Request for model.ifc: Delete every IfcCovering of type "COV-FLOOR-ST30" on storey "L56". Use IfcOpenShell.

First a look at what the model holds.

```python
import ifcopenshell
import ifcopenshell.util.element

model = ifcopenshell.open("model.ifc")
print(model.schema)
storey = next(s for s in model.by_type("IfcBuildingStorey") if s.Name == "L56")
coverings = [e for e in ifcopenshell.util.element.get_decomposition(storey) if e.is_a("IfcCovering")]
seen = {}
for e in coverings:
    element_type = ifcopenshell.util.element.get_type(e)
    name = element_type.Name if element_type not in (None, e) else None
    seen[name] = seen.get(name, 0) + 1
for name, count in sorted(seen.items(), key=str):
    print(count, "x", name)
```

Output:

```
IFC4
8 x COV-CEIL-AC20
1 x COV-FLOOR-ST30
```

```python
import ifcopenshell
import ifcopenshell.api.root
import ifcopenshell.util.element

model = ifcopenshell.open("model.ifc")

storey = next(s for s in model.by_type("IfcBuildingStorey") if s.Name == "L56")
coverings = [e for e in ifcopenshell.util.element.get_decomposition(storey) if e.is_a("IfcCovering")]
targets = [e for e in coverings if (t := ifcopenshell.util.element.get_type(e)) not in (None, e) and t.Name == "COV-FLOOR-ST30"]

for e in targets:
    ifcopenshell.api.root.remove_product(model, product=e)
print(len(targets), "removed")

model.write("model-out.ifc")
```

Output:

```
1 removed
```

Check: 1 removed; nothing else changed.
